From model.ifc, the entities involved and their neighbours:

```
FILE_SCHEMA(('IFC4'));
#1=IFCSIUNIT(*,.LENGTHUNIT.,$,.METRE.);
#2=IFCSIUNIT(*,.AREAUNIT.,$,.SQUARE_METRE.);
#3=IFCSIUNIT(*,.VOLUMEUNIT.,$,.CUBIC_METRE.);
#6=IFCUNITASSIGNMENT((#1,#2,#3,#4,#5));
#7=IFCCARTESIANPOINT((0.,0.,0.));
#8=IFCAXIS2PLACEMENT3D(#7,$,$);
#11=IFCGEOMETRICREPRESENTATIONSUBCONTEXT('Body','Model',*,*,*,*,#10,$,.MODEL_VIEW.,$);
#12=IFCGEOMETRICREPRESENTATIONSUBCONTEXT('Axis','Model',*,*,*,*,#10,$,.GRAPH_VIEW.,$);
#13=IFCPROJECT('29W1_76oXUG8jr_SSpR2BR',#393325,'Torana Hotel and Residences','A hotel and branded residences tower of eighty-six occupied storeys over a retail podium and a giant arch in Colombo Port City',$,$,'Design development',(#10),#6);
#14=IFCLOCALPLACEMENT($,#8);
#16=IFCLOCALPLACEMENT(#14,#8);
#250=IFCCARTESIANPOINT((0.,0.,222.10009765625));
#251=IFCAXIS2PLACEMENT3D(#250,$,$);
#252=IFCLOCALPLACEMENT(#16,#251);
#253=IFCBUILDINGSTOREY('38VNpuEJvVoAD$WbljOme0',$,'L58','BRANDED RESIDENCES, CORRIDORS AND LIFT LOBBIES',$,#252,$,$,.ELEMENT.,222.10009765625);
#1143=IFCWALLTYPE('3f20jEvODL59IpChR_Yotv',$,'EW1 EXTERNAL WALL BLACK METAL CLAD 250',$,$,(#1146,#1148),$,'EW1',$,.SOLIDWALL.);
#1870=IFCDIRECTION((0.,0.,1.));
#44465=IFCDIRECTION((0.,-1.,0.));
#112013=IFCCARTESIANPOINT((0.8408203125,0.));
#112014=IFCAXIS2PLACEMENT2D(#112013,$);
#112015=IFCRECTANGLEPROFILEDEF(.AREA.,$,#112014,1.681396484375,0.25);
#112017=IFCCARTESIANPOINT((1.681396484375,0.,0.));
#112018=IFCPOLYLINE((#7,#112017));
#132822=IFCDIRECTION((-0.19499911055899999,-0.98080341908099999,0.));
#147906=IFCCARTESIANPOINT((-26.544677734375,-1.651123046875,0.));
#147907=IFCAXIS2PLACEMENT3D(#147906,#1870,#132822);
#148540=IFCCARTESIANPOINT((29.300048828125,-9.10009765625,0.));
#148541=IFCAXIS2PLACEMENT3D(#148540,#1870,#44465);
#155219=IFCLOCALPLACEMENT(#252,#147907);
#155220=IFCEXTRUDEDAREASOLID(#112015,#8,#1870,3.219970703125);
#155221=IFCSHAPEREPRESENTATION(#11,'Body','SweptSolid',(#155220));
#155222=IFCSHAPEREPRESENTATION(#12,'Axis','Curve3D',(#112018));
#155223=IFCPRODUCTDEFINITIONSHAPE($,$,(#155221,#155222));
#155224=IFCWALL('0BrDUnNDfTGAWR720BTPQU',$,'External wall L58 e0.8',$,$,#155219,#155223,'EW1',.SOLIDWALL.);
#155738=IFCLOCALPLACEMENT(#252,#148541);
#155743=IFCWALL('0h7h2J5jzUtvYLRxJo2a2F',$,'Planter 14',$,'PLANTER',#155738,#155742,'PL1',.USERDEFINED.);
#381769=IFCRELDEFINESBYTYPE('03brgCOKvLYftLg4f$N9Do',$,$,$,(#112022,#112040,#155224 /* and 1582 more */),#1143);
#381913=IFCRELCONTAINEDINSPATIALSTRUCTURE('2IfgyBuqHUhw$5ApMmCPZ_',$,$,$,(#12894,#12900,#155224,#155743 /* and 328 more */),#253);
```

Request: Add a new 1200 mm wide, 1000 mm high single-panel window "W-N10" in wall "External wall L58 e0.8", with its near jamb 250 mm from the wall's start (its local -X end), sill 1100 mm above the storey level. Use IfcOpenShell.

```python
import numpy as np
import ifcopenshell
import ifcopenshell.api.feature
import ifcopenshell.api.geometry
import ifcopenshell.api.root
import ifcopenshell.api.spatial
import ifcopenshell.geom
import ifcopenshell.util.element
import ifcopenshell.util.placement
import ifcopenshell.util.representation
import ifcopenshell.util.shape
import ifcopenshell.util.unit

model = ifcopenshell.open("model.ifc")
unit_scale = ifcopenshell.util.unit.calculate_unit_scale(model)
settings = ifcopenshell.geom.settings()


def volume(element):
    """Net volume in cubic metres, openings subtracted."""
    shape = ifcopenshell.geom.create_shape(settings, element)
    return ifcopenshell.util.shape.get_volume(shape.geometry)


wall = model.by_guid("0BrDUnNDfTGAWR720BTPQU")
storey = ifcopenshell.util.element.get_container(wall, ifc_class="IfcBuildingStorey")
context = ifcopenshell.util.representation.get_context(model, "Model", "Body", "MODEL_VIEW")
before = volume(wall)

width, height, from_end, sill = 1.2, 1, 0.25, 1.1  # metres

# The wall runs along its own X axis, and the end named is its -X end.
wall_shape = ifcopenshell.geom.create_shape(settings, wall)
x, y, z = ifcopenshell.util.shape.get_vertices(wall_shape.geometry).T
start = x.min() + from_end
face, thickness = float(y.min()), float(y.max() - y.min())
wall_matrix = ifcopenshell.util.placement.get_local_placement(wall.ObjectPlacement)
level = ifcopenshell.util.placement.get_local_placement(storey.ObjectPlacement)[2, 3]


def in_wall(x, y):
    """Placement at x, y metres in the wall's axes, at sill height."""
    matrix = wall_matrix.copy()
    matrix[:, 3] = wall_matrix @ np.array([x / unit_scale, y / unit_scale, 0.0, 1.0])
    matrix[2, 3] = level + sill / unit_scale
    return matrix


# Opening: a box that overshoots both wall faces by 50 mm.
opening = ifcopenshell.api.root.create_entity(model, ifc_class="IfcOpeningElement", predefined_type="OPENING")
box = ifcopenshell.api.geometry.add_wall_representation(
    model, context=context, length=width, height=height, thickness=thickness + 0.1
)
ifcopenshell.api.geometry.assign_representation(model, product=opening, representation=box)
ifcopenshell.api.geometry.edit_object_placement(model, product=opening, matrix=in_wall(start, face - 0.05), is_si=False)
ifcopenshell.api.feature.add_feature(model, feature=opening, element=wall)

window = ifcopenshell.api.root.create_entity(model, ifc_class="IfcWindow", name="W-N10", predefined_type="WINDOW")
window.OverallWidth, window.OverallHeight = width / unit_scale, height / unit_scale
window.PartitioningType = "SINGLE_PANEL"
body = ifcopenshell.api.geometry.add_window_representation(
    model,
    context=context,
    overall_width=window.OverallWidth,
    overall_height=window.OverallHeight,
    partition_type="SINGLE_PANEL",
)
ifcopenshell.api.geometry.assign_representation(model, product=window, representation=body)
ifcopenshell.api.spatial.assign_container(model, products=[window], relating_structure=storey)
ifcopenshell.api.feature.add_filling(model, opening=opening, element=window)

# Centre the window in the wall's thickness.
ifcopenshell.api.geometry.edit_object_placement(model, product=window, matrix=in_wall(start, face), is_si=False)
window_shape = ifcopenshell.geom.create_shape(settings, window)
depth = ifcopenshell.util.shape.get_vertices(window_shape.geometry)[:, 1]
offset = face + thickness / 2 - (depth.min() + depth.max()) / 2
ifcopenshell.api.geometry.edit_object_placement(model, product=window, matrix=in_wall(start, offset), is_si=False)

after = volume(wall)

print(f"wall volume {before:.3f} -> {after:.3f} m3")

model.write("model-out.ifc")
```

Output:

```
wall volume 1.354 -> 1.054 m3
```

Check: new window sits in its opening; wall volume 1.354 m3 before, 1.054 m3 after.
